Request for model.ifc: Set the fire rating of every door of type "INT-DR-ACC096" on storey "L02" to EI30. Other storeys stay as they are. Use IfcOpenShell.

First a look at what the model holds.

```python
import ifcopenshell
import ifcopenshell.util.element

model = ifcopenshell.open("model.ifc")
print(model.schema)
storey = next(s for s in model.by_type("IfcBuildingStorey") if s.Name == "L02")
doors = [e for e in ifcopenshell.util.element.get_decomposition(storey) if e.is_a("IfcDoor")]
seen = {}
for e in doors:
    element_type = ifcopenshell.util.element.get_type(e)
    key = (element_type.Name if element_type != e and element_type else None, ifcopenshell.util.element.get_pset(e, "Pset_DoorCommon", "FireRating"))
    seen[key] = seen.get(key, 0) + 1
for (name, value), count in sorted(seen.items(), key=str):
    print(count, "x", name, "|", value)
```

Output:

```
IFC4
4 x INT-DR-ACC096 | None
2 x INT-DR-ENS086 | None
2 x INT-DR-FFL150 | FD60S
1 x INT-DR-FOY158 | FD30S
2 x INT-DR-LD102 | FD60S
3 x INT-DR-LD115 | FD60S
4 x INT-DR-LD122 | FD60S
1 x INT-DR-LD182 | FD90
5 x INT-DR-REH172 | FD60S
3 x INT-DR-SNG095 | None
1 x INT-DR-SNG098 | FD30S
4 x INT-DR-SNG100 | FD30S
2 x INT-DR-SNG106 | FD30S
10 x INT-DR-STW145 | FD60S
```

```python
import ifcopenshell
import ifcopenshell.api.pset
import ifcopenshell.util.element

model = ifcopenshell.open("model.ifc")

storey = next(s for s in model.by_type("IfcBuildingStorey") if s.Name == "L02")
doors = [e for e in ifcopenshell.util.element.get_decomposition(storey) if e.is_a("IfcDoor")]

count = 0
for e in doors:
    element_type = ifcopenshell.util.element.get_type(e)
    if element_type in (None, e) or element_type.Name != "INT-DR-ACC096":
        continue
    # add_pset returns the element's existing set when there is one.
    pset = ifcopenshell.api.pset.add_pset(model, product=e, name="Pset_DoorCommon")
    ifcopenshell.api.pset.edit_pset(model, pset=pset, properties={"FireRating": "EI30"})
    count += 1

print(count, "doors updated")

model.write("model_rev.ifc")
```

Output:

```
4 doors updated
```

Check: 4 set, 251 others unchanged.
